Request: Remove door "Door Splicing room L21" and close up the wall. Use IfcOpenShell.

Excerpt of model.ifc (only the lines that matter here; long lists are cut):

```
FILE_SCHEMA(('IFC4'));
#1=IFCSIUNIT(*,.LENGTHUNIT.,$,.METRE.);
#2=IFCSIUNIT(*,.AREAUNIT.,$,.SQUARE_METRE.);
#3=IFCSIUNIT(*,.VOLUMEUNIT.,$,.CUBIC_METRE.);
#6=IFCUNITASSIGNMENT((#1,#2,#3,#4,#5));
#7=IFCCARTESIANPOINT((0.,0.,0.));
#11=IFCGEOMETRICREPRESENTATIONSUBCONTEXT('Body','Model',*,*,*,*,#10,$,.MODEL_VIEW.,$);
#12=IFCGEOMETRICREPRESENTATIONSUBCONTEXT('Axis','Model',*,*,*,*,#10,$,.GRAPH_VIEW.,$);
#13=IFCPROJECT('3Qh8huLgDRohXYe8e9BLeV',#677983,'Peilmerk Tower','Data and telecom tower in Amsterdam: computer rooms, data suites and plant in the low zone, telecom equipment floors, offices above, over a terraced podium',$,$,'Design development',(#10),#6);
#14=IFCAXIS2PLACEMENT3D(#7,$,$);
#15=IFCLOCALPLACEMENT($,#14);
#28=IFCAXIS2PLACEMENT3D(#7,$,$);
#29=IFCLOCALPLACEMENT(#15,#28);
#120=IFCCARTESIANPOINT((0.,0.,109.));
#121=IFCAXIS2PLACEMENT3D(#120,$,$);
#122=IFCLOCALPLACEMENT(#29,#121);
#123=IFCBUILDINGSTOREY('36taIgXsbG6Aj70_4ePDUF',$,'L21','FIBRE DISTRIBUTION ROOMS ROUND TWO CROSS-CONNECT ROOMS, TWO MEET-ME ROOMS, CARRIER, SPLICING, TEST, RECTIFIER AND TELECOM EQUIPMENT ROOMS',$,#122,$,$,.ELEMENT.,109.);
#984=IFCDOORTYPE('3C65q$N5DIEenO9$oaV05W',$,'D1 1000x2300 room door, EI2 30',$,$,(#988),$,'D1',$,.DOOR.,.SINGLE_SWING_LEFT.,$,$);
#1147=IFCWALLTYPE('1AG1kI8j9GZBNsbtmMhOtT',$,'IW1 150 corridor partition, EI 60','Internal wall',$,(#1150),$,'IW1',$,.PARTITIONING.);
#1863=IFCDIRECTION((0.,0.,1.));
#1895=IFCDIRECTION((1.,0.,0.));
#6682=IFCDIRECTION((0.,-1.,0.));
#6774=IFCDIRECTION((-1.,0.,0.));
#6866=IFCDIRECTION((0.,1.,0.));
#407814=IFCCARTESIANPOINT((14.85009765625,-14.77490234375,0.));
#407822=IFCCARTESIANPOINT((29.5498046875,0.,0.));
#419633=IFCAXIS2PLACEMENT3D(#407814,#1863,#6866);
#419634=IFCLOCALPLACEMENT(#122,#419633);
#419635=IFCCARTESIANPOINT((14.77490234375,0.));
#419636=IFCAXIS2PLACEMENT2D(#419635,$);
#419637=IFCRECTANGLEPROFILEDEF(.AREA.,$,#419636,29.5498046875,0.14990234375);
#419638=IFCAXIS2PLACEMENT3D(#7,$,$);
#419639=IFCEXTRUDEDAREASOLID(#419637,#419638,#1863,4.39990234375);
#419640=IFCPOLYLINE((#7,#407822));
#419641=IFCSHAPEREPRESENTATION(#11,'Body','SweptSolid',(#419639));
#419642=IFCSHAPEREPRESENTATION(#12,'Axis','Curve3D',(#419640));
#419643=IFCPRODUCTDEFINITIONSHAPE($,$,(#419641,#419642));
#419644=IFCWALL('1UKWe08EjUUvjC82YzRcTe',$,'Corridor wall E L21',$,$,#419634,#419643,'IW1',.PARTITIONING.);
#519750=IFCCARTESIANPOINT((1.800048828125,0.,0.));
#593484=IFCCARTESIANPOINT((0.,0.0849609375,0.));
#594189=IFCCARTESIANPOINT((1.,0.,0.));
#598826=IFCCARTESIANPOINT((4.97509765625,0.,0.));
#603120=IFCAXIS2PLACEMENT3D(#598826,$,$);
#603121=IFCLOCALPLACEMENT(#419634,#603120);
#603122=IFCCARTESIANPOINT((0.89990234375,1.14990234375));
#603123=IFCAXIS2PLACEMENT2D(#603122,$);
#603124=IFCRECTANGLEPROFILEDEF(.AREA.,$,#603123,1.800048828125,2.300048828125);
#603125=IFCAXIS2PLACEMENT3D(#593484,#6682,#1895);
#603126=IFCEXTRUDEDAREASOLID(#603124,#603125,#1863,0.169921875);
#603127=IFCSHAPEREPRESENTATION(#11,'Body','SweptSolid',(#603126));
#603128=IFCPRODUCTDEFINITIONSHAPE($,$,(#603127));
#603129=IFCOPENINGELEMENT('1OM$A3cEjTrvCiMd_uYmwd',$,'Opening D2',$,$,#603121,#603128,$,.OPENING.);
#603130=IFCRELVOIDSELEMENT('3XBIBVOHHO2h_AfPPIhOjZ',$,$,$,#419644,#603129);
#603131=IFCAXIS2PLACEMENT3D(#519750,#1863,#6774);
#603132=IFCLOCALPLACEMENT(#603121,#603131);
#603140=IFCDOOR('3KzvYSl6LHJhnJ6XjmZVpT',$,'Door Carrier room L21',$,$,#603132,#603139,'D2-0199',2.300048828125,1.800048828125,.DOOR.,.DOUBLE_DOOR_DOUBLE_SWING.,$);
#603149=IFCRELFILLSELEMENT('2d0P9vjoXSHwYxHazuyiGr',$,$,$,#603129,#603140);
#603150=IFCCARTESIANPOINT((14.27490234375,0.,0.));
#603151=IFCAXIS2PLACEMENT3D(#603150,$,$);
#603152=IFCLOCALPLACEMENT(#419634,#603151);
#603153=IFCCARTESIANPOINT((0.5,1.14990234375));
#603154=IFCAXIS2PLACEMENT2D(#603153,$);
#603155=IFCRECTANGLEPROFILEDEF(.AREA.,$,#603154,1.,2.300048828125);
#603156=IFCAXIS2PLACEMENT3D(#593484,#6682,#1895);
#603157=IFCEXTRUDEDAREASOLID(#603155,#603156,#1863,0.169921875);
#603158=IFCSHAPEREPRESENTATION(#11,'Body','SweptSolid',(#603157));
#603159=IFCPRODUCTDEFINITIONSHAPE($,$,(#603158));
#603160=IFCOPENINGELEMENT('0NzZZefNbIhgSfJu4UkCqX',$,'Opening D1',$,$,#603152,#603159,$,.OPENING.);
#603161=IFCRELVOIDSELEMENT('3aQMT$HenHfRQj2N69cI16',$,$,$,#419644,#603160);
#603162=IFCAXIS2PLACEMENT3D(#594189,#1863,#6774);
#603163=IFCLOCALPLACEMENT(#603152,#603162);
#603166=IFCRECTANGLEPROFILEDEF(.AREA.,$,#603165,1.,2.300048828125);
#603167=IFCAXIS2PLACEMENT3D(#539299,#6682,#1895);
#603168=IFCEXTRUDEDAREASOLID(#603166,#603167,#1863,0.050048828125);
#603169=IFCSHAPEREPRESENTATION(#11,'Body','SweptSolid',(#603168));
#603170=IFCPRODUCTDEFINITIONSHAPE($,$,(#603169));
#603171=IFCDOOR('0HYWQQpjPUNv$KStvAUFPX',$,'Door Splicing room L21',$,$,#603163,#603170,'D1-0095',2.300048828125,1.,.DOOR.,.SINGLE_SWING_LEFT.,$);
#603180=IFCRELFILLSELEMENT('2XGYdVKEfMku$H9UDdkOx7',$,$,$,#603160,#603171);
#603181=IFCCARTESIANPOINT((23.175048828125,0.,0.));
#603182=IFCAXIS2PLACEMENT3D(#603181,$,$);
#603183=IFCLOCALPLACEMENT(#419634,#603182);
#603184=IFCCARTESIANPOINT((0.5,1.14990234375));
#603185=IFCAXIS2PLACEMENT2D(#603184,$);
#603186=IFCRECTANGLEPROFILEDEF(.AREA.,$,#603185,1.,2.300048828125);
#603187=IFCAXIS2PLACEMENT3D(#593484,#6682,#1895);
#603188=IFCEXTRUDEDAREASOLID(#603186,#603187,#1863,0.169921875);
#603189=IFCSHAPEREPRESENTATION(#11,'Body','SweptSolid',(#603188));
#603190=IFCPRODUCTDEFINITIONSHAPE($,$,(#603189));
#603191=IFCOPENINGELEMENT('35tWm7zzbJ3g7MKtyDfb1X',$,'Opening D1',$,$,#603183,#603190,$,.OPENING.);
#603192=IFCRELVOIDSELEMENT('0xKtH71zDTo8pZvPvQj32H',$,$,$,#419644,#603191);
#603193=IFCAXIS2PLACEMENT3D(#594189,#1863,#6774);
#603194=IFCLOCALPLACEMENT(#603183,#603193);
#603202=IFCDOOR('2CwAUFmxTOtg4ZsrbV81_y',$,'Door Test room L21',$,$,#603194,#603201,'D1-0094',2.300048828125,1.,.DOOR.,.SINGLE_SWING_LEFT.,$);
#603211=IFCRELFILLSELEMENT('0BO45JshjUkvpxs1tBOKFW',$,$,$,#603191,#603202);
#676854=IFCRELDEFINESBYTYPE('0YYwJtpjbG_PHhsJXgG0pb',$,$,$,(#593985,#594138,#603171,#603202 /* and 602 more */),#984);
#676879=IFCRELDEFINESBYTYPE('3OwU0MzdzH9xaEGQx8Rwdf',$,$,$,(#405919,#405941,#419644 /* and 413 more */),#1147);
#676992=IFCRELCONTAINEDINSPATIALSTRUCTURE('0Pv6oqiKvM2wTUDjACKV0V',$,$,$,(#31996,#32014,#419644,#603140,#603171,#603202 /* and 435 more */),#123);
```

```python
import ifcopenshell
import ifcopenshell.api.feature
import ifcopenshell.api.root
import ifcopenshell.geom
import ifcopenshell.util.shape

model = ifcopenshell.open("model.ifc")
settings = ifcopenshell.geom.settings()


def volume(element):
    """Net volume in cubic metres, openings subtracted."""
    shape = ifcopenshell.geom.create_shape(settings, element)
    return ifcopenshell.util.shape.get_volume(shape.geometry)


door = model.by_guid("0HYWQQpjPUNv$KStvAUFPX")
opening = door.FillsVoids[0].RelatingOpeningElement
wall = opening.VoidsElements[0].RelatingBuildingElement
before = volume(wall)

ifcopenshell.api.root.remove_product(model, product=door)
ifcopenshell.api.feature.remove_feature(model, feature=opening)

after = volume(wall)

print(f"wall volume {before:.3f} -> {after:.3f} m3")

model.write("model_rev.ifc")
```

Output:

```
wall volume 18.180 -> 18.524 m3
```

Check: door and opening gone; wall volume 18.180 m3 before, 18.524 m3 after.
